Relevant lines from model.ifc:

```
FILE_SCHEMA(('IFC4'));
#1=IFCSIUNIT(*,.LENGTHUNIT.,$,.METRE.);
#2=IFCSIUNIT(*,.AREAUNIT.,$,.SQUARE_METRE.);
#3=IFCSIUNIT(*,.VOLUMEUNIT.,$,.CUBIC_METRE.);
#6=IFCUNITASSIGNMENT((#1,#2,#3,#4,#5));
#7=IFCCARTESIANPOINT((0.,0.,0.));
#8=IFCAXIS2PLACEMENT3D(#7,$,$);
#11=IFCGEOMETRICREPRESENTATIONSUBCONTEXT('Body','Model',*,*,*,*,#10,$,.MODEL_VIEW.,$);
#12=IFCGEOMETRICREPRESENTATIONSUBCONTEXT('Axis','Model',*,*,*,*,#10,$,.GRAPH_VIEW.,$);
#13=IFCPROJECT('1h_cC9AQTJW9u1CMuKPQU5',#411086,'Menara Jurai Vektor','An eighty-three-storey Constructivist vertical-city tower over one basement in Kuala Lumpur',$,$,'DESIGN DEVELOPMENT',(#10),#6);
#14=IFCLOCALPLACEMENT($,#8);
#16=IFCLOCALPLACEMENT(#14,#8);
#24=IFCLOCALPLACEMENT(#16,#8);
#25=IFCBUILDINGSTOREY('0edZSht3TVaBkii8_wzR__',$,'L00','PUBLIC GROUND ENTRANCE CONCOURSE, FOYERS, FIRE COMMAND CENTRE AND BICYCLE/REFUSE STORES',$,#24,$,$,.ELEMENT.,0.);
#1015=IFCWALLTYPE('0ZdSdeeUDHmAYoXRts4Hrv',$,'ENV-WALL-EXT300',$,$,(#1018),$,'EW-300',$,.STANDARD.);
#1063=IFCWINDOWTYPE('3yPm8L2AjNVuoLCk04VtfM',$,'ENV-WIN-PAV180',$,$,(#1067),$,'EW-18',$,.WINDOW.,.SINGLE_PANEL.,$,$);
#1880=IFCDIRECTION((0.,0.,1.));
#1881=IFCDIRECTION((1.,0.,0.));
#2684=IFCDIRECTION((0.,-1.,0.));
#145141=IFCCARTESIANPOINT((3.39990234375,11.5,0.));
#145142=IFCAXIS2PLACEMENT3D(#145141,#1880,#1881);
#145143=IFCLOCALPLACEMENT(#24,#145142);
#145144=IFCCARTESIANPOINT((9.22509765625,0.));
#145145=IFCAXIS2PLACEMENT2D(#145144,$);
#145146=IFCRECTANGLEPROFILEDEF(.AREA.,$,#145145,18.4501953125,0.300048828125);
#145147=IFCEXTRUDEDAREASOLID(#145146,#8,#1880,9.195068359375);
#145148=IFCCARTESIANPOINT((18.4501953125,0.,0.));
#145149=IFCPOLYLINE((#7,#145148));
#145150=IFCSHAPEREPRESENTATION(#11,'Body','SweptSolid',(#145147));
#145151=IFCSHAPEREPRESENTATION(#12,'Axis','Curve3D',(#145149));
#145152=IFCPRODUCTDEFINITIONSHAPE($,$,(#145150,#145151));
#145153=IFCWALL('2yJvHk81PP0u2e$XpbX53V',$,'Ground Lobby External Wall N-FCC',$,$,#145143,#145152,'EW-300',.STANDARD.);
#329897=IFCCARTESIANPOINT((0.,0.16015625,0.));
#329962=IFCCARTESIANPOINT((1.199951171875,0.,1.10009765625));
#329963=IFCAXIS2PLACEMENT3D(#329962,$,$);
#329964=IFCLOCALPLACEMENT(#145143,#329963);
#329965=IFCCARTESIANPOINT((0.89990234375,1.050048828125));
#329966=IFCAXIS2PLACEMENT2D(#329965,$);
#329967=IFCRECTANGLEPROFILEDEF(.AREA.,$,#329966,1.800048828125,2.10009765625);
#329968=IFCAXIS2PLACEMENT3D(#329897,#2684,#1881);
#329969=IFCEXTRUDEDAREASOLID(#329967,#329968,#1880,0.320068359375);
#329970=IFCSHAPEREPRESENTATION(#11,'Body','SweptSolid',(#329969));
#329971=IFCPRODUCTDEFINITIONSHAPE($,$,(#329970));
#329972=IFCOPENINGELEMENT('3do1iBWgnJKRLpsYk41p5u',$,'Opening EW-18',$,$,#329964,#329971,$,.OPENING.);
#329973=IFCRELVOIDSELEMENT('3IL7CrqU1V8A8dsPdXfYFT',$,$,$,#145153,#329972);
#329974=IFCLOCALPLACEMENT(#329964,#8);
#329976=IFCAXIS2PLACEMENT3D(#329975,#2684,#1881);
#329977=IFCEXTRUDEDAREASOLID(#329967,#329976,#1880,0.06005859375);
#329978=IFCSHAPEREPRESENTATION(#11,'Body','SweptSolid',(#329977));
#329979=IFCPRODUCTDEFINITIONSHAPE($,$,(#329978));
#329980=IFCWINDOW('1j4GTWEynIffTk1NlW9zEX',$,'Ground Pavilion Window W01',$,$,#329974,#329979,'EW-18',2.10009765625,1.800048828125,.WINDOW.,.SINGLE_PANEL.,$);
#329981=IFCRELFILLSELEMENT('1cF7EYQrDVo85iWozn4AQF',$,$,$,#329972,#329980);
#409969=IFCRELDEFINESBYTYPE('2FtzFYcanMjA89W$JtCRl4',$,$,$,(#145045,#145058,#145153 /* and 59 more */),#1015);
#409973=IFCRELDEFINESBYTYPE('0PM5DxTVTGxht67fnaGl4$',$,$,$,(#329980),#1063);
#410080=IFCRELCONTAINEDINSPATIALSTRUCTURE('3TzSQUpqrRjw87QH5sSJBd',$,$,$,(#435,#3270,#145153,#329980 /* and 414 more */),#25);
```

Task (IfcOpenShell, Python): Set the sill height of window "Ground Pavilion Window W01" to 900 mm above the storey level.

```python
import numpy as np
import ifcopenshell
import ifcopenshell.api.geometry
import ifcopenshell.geom
import ifcopenshell.util.element
import ifcopenshell.util.placement
import ifcopenshell.util.shape
import ifcopenshell.util.unit

model = ifcopenshell.open("model.ifc")
unit_scale = ifcopenshell.util.unit.calculate_unit_scale(model)

window = model.by_id(329980)
opening = window.FillsVoids[0].RelatingOpeningElement
storey = ifcopenshell.util.element.get_container(window, ifc_class="IfcBuildingStorey")
level = ifcopenshell.util.placement.get_local_placement(storey.ObjectPlacement)[2, 3]

# The opening's origin need not be at the sill, so measure its lowest point.
shape = ifcopenshell.geom.create_shape(ifcopenshell.geom.settings(), opening)
bottom = ifcopenshell.util.shape.get_shape_bottom_elevation(shape, shape.geometry) / unit_scale
dz = level + 0.9 / unit_scale - bottom

shift = np.array([0.0, 0.0, dz])
# The window is placed relative to its opening, so it follows when the opening moves.
matrix = ifcopenshell.util.placement.get_local_placement(opening.ObjectPlacement)
matrix[:3, 3] += shift
ifcopenshell.api.geometry.edit_object_placement(
    model, product=opening, matrix=matrix, is_si=False, should_transform_children=True
)

print(f"moved by {dz * unit_scale:+.3f} m")

model.write("model-out.ifc")
```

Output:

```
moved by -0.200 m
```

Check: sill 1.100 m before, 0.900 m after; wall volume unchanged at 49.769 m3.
